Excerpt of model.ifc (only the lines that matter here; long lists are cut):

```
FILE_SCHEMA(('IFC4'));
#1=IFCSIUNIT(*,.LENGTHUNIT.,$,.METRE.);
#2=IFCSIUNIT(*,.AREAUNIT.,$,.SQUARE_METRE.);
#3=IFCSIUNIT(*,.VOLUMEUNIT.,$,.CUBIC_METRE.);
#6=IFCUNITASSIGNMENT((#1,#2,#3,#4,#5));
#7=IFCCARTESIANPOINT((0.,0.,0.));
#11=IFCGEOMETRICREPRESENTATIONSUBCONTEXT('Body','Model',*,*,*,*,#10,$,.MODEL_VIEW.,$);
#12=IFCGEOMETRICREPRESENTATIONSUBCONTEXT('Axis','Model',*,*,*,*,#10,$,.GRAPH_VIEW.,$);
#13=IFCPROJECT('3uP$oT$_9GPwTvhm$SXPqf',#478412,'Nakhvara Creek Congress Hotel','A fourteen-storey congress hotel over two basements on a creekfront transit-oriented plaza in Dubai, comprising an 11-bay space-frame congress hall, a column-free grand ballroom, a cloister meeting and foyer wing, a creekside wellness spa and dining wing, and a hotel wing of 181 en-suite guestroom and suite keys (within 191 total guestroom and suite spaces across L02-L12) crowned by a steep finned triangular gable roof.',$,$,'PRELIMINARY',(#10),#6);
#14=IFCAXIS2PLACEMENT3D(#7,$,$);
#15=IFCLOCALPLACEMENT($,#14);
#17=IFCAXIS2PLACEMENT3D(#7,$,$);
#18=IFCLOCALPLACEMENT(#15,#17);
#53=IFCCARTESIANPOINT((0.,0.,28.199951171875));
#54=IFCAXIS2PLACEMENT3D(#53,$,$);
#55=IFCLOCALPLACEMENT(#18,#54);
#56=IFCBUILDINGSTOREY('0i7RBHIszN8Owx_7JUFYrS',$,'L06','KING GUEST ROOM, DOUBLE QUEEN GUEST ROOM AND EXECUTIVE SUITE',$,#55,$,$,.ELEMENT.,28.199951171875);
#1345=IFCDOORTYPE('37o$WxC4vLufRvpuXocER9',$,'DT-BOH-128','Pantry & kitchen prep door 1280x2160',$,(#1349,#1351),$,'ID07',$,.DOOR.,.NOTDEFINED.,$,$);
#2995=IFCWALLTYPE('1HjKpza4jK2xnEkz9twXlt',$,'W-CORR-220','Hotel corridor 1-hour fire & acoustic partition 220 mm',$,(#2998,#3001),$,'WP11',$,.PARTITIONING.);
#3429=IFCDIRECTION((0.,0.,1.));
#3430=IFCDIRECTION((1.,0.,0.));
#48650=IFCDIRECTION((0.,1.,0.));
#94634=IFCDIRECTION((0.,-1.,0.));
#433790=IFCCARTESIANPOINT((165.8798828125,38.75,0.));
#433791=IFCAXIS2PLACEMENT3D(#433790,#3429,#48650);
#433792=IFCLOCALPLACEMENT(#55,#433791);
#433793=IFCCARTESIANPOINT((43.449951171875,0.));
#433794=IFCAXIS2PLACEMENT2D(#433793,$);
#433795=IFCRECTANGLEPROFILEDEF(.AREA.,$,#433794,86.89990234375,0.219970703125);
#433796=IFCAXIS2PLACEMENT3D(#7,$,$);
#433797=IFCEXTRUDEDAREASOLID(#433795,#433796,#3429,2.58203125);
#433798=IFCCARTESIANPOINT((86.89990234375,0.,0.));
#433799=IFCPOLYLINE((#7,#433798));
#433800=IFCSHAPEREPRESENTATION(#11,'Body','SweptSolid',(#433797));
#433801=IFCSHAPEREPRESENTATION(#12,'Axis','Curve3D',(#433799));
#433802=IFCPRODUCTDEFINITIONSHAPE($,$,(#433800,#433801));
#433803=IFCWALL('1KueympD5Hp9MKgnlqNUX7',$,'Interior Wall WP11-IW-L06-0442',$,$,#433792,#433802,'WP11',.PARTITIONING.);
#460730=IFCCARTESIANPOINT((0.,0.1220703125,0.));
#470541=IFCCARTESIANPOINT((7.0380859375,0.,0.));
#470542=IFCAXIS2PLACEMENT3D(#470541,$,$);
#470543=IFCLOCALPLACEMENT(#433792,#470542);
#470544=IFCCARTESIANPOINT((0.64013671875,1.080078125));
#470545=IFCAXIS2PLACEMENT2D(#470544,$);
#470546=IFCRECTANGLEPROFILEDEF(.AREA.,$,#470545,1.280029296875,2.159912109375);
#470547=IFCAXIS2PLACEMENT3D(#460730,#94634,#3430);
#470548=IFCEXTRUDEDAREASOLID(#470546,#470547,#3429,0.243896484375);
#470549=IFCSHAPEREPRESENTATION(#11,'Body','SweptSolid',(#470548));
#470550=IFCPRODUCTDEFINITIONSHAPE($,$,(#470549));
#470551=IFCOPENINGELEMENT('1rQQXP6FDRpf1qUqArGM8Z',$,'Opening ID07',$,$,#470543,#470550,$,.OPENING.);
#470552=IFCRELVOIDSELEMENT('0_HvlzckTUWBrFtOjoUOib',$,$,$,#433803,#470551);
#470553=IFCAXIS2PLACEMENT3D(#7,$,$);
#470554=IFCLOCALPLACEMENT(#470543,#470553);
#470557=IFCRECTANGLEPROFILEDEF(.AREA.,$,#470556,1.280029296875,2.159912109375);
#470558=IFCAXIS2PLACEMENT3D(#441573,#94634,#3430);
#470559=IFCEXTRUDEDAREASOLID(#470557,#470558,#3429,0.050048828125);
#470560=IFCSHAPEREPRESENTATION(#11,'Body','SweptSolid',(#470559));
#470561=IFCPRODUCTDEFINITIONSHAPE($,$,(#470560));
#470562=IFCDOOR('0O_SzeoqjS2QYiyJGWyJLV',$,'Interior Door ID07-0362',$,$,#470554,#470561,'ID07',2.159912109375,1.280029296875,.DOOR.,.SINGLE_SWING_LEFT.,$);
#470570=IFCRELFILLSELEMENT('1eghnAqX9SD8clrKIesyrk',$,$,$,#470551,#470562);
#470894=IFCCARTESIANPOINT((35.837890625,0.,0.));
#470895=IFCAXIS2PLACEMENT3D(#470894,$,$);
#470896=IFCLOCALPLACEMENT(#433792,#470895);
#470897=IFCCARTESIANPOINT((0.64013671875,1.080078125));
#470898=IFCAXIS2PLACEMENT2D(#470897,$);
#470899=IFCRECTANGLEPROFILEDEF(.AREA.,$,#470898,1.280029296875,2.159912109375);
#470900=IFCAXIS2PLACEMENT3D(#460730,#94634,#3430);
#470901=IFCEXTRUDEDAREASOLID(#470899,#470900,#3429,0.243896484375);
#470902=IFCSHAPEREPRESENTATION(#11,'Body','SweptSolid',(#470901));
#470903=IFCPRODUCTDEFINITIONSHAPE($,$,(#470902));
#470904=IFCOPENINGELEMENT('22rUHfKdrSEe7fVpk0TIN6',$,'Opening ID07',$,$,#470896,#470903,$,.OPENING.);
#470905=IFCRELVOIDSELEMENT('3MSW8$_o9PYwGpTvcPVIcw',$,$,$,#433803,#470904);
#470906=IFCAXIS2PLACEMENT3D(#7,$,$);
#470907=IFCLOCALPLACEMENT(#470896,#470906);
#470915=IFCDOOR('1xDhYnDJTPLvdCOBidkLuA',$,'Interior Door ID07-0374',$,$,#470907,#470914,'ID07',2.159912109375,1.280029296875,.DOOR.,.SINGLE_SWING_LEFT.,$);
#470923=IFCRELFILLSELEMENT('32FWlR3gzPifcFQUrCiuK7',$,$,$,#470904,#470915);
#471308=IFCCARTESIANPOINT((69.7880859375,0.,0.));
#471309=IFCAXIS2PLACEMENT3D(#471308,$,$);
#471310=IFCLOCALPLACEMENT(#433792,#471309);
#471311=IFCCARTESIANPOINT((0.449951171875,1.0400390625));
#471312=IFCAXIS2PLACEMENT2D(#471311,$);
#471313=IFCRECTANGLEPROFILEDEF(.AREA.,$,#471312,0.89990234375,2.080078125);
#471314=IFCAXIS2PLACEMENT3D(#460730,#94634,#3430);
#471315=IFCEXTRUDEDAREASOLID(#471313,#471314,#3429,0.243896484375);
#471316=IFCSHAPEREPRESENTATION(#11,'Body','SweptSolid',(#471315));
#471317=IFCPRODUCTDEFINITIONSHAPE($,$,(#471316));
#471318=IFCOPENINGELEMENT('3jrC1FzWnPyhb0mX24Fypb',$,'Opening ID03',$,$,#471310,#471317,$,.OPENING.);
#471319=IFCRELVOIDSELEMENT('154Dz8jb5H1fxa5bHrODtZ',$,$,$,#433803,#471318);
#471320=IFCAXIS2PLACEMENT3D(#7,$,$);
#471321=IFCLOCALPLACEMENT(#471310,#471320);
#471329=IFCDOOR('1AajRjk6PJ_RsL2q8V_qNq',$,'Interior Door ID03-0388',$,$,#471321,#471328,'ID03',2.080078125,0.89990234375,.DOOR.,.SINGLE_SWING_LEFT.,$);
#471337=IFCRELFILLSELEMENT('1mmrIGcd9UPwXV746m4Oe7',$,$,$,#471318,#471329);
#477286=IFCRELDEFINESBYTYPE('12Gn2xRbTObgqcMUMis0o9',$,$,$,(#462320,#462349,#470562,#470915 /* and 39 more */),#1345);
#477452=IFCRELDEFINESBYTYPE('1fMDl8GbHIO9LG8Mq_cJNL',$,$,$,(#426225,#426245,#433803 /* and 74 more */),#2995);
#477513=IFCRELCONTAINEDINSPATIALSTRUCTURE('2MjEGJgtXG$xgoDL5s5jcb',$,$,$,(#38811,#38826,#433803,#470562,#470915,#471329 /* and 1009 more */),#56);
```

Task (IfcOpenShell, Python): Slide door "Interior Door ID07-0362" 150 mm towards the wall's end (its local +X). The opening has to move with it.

```python
import ifcopenshell
import ifcopenshell.api.geometry
import ifcopenshell.util.placement

model = ifcopenshell.open("model.ifc")

door = model.by_guid("0O_SzeoqjS2QYiyJGWyJLV")
opening = door.FillsVoids[0].RelatingOpeningElement
wall = opening.VoidsElements[0].RelatingBuildingElement

wall_matrix = ifcopenshell.util.placement.get_local_placement(wall.ObjectPlacement)
shift = wall_matrix[:3, 0] * 0.15
before = ifcopenshell.util.placement.get_local_placement(door.ObjectPlacement)[:3, 3].copy()

# The door is placed relative to its opening, so it follows when the opening moves.
matrix = ifcopenshell.util.placement.get_local_placement(opening.ObjectPlacement)
matrix[:3, 3] += shift
ifcopenshell.api.geometry.edit_object_placement(
    model, product=opening, matrix=matrix, is_si=False, should_transform_children=True
)

after = ifcopenshell.util.placement.get_local_placement(door.ObjectPlacement)[:3, 3]
print("door moved by", (after - before).round(3) + 0.0)

model.write("model_v2.ifc")
```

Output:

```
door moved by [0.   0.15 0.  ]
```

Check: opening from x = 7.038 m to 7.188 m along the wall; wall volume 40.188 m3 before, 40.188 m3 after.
